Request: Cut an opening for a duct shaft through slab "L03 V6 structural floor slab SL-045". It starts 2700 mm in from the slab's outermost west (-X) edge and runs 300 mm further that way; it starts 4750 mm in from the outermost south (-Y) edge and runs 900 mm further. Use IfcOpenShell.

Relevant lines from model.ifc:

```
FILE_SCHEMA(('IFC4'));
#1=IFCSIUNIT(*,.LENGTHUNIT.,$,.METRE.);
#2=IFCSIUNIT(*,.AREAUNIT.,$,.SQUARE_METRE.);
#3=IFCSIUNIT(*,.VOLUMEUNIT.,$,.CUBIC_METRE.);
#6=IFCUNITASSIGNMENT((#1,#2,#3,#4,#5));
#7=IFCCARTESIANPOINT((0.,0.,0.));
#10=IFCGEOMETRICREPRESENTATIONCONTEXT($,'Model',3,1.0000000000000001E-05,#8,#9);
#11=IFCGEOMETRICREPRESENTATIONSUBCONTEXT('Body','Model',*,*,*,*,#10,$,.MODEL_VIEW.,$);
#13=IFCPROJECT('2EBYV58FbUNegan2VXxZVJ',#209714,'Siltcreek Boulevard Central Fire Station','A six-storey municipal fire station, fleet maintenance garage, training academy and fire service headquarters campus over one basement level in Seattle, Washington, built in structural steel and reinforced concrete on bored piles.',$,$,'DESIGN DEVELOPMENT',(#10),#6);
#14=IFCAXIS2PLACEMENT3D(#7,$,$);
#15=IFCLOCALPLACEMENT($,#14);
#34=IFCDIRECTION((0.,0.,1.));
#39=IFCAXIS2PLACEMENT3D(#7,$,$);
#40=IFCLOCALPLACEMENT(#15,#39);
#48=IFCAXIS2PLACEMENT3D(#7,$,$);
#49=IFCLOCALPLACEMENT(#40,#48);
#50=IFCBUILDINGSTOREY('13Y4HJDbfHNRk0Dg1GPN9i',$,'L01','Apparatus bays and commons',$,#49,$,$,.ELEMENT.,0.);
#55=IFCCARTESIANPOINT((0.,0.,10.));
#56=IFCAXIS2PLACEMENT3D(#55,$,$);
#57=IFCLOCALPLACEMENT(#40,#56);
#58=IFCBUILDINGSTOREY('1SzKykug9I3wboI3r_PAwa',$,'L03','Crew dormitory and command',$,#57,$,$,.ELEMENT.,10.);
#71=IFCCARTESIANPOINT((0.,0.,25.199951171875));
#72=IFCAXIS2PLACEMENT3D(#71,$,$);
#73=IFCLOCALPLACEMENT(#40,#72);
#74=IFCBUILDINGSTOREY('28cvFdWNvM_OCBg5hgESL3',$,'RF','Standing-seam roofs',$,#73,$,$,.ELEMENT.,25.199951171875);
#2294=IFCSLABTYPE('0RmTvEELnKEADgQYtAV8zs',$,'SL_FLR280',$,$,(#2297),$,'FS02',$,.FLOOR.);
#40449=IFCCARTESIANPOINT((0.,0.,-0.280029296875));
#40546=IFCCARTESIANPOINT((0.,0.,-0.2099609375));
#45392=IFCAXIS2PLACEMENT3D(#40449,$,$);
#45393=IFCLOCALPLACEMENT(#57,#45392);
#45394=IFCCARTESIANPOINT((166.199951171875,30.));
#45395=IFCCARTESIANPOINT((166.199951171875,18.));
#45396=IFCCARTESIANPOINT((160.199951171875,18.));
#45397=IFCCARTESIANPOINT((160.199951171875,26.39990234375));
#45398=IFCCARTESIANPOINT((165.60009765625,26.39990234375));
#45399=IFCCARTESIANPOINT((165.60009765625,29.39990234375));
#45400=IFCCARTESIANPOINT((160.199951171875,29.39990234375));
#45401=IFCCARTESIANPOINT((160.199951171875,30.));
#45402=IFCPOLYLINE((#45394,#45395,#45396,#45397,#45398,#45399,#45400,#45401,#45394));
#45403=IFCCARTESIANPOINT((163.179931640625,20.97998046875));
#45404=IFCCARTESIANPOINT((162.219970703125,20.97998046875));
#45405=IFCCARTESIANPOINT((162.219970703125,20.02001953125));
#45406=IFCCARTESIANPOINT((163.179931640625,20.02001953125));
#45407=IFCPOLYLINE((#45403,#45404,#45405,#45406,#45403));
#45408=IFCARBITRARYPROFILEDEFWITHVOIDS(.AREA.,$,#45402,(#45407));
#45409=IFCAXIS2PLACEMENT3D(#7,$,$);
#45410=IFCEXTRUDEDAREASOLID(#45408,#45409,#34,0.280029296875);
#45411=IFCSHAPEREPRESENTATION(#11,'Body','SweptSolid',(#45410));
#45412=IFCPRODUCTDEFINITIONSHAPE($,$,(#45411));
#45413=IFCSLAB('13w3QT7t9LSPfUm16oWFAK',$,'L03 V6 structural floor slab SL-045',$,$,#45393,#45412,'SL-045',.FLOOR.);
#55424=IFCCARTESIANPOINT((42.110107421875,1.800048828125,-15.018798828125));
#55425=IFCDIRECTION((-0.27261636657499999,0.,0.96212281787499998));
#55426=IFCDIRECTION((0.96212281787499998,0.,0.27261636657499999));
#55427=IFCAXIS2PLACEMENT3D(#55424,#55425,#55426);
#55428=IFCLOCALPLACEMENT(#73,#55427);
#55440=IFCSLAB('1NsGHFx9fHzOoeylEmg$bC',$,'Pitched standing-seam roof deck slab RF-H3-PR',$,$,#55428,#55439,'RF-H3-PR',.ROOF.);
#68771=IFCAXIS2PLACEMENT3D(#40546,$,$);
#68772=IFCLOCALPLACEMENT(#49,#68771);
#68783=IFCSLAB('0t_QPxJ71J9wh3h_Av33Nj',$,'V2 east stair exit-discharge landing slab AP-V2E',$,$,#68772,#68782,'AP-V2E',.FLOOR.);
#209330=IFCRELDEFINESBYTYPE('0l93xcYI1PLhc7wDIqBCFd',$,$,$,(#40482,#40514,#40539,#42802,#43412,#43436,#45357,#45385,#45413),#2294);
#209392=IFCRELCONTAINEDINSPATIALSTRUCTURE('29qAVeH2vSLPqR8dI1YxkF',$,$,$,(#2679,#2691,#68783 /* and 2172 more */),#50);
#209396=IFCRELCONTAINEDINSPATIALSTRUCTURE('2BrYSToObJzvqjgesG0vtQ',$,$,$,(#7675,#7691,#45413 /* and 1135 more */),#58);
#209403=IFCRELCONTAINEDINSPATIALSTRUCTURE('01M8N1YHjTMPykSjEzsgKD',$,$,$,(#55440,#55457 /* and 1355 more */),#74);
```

```python
import numpy as np
import ifcopenshell
import ifcopenshell.api.feature
import ifcopenshell.api.geometry
import ifcopenshell.api.root
import ifcopenshell.geom
import ifcopenshell.util.placement
import ifcopenshell.util.representation
import ifcopenshell.util.shape
import ifcopenshell.util.unit

model = ifcopenshell.open("model.ifc")
unit_scale = ifcopenshell.util.unit.calculate_unit_scale(model)
settings = ifcopenshell.geom.settings()


def volume(element):
    """Net volume in cubic metres, openings subtracted."""
    shape = ifcopenshell.geom.create_shape(settings, element)
    return ifcopenshell.util.shape.get_volume(shape.geometry)


slab = model.by_guid("13w3QT7t9LSPfUm16oWFAK")
before = volume(slab)

# Extent in the slab's own axes, in metres. The edges named are its -X and -Y sides.
slab_shape = ifcopenshell.geom.create_shape(settings, slab)
vertices = ifcopenshell.util.shape.get_vertices(slab_shape.geometry)
x_min, y_min, bottom = vertices.min(axis=0)
top = vertices[:, 2].max()

opening = ifcopenshell.api.root.create_entity(model, ifc_class="IfcOpeningElement", name="Duct shaft opening", predefined_type="OPENING")
context = ifcopenshell.util.representation.get_context(model, "Model", "Body", "MODEL_VIEW")
width, depth = 0.3, 0.9
outline = [(0.0, 0.0), (width, 0.0), (width, depth), (0.0, depth), (0.0, 0.0)]
# Overshoot both faces by 50 mm so the cut is clean.
shape = ifcopenshell.api.geometry.add_slab_representation(
    model, context=context, depth=top - bottom + 0.1, polyline=outline
)
ifcopenshell.api.geometry.assign_representation(model, product=opening, representation=shape)

matrix = ifcopenshell.util.placement.get_local_placement(slab.ObjectPlacement)
matrix[:, 3] = matrix @ np.append(np.array([x_min + 2.7, y_min + 4.75, bottom - 0.05]) / unit_scale, 1.0)
ifcopenshell.api.geometry.edit_object_placement(model, product=opening, matrix=matrix, is_si=False)
ifcopenshell.api.feature.add_feature(model, feature=opening, element=slab)

after = volume(slab)

print(f"slab volume {before:.3f} -> {after:.3f} m3")

model.write("model-out.ifc")
```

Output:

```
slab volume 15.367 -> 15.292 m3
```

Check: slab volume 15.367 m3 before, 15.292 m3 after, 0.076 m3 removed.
